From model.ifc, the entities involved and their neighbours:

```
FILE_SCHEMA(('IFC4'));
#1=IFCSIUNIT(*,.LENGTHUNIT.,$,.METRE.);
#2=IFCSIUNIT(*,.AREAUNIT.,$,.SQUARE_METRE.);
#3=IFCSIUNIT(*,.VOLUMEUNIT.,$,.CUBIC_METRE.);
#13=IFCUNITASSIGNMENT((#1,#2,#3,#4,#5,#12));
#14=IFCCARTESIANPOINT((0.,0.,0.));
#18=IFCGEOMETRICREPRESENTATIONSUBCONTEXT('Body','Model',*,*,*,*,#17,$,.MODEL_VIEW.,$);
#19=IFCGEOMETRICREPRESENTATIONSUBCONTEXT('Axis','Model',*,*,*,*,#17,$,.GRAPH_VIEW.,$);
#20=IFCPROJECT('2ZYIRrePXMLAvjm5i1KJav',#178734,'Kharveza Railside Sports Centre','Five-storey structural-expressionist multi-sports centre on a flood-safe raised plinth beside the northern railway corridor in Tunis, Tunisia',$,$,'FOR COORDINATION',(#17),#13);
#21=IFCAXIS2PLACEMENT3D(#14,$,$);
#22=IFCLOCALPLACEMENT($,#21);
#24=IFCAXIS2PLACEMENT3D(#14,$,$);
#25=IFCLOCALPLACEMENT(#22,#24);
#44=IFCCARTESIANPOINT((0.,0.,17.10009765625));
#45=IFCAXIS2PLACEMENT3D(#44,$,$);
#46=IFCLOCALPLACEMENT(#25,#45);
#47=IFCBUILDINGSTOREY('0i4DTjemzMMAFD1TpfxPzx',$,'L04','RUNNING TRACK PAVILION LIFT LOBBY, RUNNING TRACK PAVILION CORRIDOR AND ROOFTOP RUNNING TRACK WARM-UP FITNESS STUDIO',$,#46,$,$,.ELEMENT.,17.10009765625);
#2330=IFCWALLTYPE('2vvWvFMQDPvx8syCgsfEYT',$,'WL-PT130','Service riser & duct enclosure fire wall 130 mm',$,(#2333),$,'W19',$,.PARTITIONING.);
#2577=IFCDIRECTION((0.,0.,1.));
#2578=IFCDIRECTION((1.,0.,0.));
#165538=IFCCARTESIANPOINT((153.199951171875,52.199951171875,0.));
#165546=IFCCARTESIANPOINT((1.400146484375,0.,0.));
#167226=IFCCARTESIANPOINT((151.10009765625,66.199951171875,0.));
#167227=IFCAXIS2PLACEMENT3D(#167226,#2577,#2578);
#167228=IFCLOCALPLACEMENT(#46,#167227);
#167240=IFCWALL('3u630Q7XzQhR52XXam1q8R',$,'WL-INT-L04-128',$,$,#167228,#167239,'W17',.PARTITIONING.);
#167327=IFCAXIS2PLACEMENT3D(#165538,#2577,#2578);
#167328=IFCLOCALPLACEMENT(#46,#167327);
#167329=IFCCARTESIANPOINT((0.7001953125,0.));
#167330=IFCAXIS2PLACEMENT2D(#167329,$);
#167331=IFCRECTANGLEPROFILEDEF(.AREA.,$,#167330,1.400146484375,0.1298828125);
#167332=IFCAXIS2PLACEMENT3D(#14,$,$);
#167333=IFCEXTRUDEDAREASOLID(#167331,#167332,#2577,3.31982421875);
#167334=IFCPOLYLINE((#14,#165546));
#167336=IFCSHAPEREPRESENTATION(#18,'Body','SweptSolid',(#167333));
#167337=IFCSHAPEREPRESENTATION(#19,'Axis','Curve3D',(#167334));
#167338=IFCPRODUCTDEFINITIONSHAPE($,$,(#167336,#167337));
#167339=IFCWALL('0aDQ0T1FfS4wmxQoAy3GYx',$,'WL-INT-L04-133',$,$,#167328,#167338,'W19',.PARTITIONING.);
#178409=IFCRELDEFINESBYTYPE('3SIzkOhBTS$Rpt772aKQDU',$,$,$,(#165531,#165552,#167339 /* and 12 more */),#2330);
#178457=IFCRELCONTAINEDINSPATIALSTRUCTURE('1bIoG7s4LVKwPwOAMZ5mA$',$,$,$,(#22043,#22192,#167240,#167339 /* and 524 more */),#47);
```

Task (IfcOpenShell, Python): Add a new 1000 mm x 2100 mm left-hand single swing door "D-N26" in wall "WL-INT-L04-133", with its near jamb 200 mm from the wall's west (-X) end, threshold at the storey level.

```python
import numpy as np
import ifcopenshell
import ifcopenshell.api.feature
import ifcopenshell.api.geometry
import ifcopenshell.api.root
import ifcopenshell.api.spatial
import ifcopenshell.geom
import ifcopenshell.util.element
import ifcopenshell.util.placement
import ifcopenshell.util.representation
import ifcopenshell.util.shape
import ifcopenshell.util.unit

model = ifcopenshell.open("model.ifc")
unit_scale = ifcopenshell.util.unit.calculate_unit_scale(model)
settings = ifcopenshell.geom.settings()


def volume(element):
    """Net volume in cubic metres, openings subtracted."""
    shape = ifcopenshell.geom.create_shape(settings, element)
    return ifcopenshell.util.shape.get_volume(shape.geometry)


wall = model.by_guid("0aDQ0T1FfS4wmxQoAy3GYx")
storey = ifcopenshell.util.element.get_container(wall, ifc_class="IfcBuildingStorey")
context = ifcopenshell.util.representation.get_context(model, "Model", "Body", "MODEL_VIEW")
before = volume(wall)

width, height, from_end, sill = 1, 2.1, 0.2, 0.0  # metres

# The wall runs along its own X axis, and the end named is its -X end.
wall_shape = ifcopenshell.geom.create_shape(settings, wall)
x, y, z = ifcopenshell.util.shape.get_vertices(wall_shape.geometry).T
start = x.min() + from_end
face, thickness = float(y.min()), float(y.max() - y.min())
wall_matrix = ifcopenshell.util.placement.get_local_placement(wall.ObjectPlacement)
level = ifcopenshell.util.placement.get_local_placement(storey.ObjectPlacement)[2, 3]


def in_wall(x, y):
    """Placement at x, y metres in the wall's axes, at sill height."""
    matrix = wall_matrix.copy()
    matrix[:, 3] = wall_matrix @ np.array([x / unit_scale, y / unit_scale, 0.0, 1.0])
    matrix[2, 3] = level + sill / unit_scale
    return matrix


# Opening: a box that overshoots both wall faces by 50 mm.
opening = ifcopenshell.api.root.create_entity(model, ifc_class="IfcOpeningElement", predefined_type="OPENING")
box = ifcopenshell.api.geometry.add_wall_representation(
    model, context=context, length=width, height=height, thickness=thickness + 0.1
)
ifcopenshell.api.geometry.assign_representation(model, product=opening, representation=box)
ifcopenshell.api.geometry.edit_object_placement(model, product=opening, matrix=in_wall(start, face - 0.05), is_si=False)
ifcopenshell.api.feature.add_feature(model, feature=opening, element=wall)

door = ifcopenshell.api.root.create_entity(model, ifc_class="IfcDoor", name="D-N26", predefined_type="DOOR")
door.OverallWidth, door.OverallHeight = width / unit_scale, height / unit_scale
door.OperationType = "SINGLE_SWING_LEFT"
body = ifcopenshell.api.geometry.add_door_representation(
    model,
    context=context,
    overall_width=door.OverallWidth,
    overall_height=door.OverallHeight,
    operation_type="SINGLE_SWING_LEFT",
    lining_properties={"LiningDepth": thickness / unit_scale, "ThresholdDepth": thickness / unit_scale},
)
ifcopenshell.api.geometry.assign_representation(model, product=door, representation=body)
ifcopenshell.api.spatial.assign_container(model, products=[door], relating_structure=storey)
ifcopenshell.api.feature.add_filling(model, opening=opening, element=door)

# The lining spans the wall, so the door starts at the wall face.
ifcopenshell.api.geometry.edit_object_placement(model, product=door, matrix=in_wall(start, face), is_si=False)

after = volume(wall)

print(f"wall volume {before:.3f} -> {after:.3f} m3")

model.write("model_v2.ifc")
```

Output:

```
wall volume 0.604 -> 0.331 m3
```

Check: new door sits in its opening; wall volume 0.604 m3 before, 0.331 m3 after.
